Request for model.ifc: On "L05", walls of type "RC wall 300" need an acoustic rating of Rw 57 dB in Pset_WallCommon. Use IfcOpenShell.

First a look at what the model holds.

```python
import ifcopenshell
import ifcopenshell.util.element

model = ifcopenshell.open("model.ifc")
print(model.schema)
storey = next(s for s in model.by_type("IfcBuildingStorey") if s.Name == "L05")
walls = [e for e in ifcopenshell.util.element.get_decomposition(storey) if e.is_a("IfcWall")]
seen = {}
for e in walls:
    element_type = ifcopenshell.util.element.get_type(e)
    key = (element_type.Name if element_type != e and element_type else None, ifcopenshell.util.element.get_pset(e, "Pset_WallCommon", "AcousticRating"))
    seen[key] = seen.get(key, 0) + 1
for (name, value), count in sorted(seen.items(), key=str):
    print(count, "x", name, "|", value)
```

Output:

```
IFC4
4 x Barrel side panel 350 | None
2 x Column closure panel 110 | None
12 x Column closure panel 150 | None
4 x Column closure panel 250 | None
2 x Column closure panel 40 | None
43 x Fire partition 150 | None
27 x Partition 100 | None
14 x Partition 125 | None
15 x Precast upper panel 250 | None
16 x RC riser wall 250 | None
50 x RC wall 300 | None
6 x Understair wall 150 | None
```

```python
import ifcopenshell
import ifcopenshell.api.pset
import ifcopenshell.util.element

model = ifcopenshell.open("model.ifc")

storey = next(s for s in model.by_type("IfcBuildingStorey") if s.Name == "L05")
walls = [e for e in ifcopenshell.util.element.get_decomposition(storey) if e.is_a("IfcWall")]

count = 0
for e in walls:
    element_type = ifcopenshell.util.element.get_type(e)
    if element_type in (None, e) or element_type.Name != "RC wall 300":
        continue
    # add_pset returns the element's existing set when there is one.
    pset = ifcopenshell.api.pset.add_pset(model, product=e, name="Pset_WallCommon")
    ifcopenshell.api.pset.edit_pset(model, pset=pset, properties={"AcousticRating": "Rw 57 dB"})
    count += 1

print(count, "walls updated")

model.write("model_edited.ifc")
```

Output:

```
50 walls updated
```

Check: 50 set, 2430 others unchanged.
